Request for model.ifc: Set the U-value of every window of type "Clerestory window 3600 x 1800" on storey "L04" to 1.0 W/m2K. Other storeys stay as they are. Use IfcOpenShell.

First a look at what the model holds.

```python
import ifcopenshell
import ifcopenshell.util.element

model = ifcopenshell.open("model.ifc")
print(model.schema)
storey = next(s for s in model.by_type("IfcBuildingStorey") if s.Name == "L04")
windows = [e for e in ifcopenshell.util.element.get_decomposition(storey) if e.is_a("IfcWindow")]
seen = {}
for e in windows:
    element_type = ifcopenshell.util.element.get_type(e)
    key = (element_type.Name if element_type != e and element_type else None, ifcopenshell.util.element.get_pset(e, "Pset_WindowCommon", "ThermalTransmittance"))
    seen[key] = seen.get(key, 0) + 1
for (name, value), count in sorted(seen.items(), key=str):
    print(count, "x", name, "|", value)
```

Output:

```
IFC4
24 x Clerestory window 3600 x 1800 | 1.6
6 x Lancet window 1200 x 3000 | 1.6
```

```python
import ifcopenshell
import ifcopenshell.api.pset
import ifcopenshell.util.element

model = ifcopenshell.open("model.ifc")

storey = next(s for s in model.by_type("IfcBuildingStorey") if s.Name == "L04")
windows = [e for e in ifcopenshell.util.element.get_decomposition(storey) if e.is_a("IfcWindow")]

count = 0
for e in windows:
    element_type = ifcopenshell.util.element.get_type(e)
    if element_type in (None, e) or element_type.Name != "Clerestory window 3600 x 1800":
        continue
    # add_pset returns the element's existing set when there is one.
    pset = ifcopenshell.api.pset.add_pset(model, product=e, name="Pset_WindowCommon")
    ifcopenshell.api.pset.edit_pset(model, pset=pset, properties={"ThermalTransmittance": 1.0})
    count += 1

print(count, "windows updated")

model.write("model-out.ifc")
```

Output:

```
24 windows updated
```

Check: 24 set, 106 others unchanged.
